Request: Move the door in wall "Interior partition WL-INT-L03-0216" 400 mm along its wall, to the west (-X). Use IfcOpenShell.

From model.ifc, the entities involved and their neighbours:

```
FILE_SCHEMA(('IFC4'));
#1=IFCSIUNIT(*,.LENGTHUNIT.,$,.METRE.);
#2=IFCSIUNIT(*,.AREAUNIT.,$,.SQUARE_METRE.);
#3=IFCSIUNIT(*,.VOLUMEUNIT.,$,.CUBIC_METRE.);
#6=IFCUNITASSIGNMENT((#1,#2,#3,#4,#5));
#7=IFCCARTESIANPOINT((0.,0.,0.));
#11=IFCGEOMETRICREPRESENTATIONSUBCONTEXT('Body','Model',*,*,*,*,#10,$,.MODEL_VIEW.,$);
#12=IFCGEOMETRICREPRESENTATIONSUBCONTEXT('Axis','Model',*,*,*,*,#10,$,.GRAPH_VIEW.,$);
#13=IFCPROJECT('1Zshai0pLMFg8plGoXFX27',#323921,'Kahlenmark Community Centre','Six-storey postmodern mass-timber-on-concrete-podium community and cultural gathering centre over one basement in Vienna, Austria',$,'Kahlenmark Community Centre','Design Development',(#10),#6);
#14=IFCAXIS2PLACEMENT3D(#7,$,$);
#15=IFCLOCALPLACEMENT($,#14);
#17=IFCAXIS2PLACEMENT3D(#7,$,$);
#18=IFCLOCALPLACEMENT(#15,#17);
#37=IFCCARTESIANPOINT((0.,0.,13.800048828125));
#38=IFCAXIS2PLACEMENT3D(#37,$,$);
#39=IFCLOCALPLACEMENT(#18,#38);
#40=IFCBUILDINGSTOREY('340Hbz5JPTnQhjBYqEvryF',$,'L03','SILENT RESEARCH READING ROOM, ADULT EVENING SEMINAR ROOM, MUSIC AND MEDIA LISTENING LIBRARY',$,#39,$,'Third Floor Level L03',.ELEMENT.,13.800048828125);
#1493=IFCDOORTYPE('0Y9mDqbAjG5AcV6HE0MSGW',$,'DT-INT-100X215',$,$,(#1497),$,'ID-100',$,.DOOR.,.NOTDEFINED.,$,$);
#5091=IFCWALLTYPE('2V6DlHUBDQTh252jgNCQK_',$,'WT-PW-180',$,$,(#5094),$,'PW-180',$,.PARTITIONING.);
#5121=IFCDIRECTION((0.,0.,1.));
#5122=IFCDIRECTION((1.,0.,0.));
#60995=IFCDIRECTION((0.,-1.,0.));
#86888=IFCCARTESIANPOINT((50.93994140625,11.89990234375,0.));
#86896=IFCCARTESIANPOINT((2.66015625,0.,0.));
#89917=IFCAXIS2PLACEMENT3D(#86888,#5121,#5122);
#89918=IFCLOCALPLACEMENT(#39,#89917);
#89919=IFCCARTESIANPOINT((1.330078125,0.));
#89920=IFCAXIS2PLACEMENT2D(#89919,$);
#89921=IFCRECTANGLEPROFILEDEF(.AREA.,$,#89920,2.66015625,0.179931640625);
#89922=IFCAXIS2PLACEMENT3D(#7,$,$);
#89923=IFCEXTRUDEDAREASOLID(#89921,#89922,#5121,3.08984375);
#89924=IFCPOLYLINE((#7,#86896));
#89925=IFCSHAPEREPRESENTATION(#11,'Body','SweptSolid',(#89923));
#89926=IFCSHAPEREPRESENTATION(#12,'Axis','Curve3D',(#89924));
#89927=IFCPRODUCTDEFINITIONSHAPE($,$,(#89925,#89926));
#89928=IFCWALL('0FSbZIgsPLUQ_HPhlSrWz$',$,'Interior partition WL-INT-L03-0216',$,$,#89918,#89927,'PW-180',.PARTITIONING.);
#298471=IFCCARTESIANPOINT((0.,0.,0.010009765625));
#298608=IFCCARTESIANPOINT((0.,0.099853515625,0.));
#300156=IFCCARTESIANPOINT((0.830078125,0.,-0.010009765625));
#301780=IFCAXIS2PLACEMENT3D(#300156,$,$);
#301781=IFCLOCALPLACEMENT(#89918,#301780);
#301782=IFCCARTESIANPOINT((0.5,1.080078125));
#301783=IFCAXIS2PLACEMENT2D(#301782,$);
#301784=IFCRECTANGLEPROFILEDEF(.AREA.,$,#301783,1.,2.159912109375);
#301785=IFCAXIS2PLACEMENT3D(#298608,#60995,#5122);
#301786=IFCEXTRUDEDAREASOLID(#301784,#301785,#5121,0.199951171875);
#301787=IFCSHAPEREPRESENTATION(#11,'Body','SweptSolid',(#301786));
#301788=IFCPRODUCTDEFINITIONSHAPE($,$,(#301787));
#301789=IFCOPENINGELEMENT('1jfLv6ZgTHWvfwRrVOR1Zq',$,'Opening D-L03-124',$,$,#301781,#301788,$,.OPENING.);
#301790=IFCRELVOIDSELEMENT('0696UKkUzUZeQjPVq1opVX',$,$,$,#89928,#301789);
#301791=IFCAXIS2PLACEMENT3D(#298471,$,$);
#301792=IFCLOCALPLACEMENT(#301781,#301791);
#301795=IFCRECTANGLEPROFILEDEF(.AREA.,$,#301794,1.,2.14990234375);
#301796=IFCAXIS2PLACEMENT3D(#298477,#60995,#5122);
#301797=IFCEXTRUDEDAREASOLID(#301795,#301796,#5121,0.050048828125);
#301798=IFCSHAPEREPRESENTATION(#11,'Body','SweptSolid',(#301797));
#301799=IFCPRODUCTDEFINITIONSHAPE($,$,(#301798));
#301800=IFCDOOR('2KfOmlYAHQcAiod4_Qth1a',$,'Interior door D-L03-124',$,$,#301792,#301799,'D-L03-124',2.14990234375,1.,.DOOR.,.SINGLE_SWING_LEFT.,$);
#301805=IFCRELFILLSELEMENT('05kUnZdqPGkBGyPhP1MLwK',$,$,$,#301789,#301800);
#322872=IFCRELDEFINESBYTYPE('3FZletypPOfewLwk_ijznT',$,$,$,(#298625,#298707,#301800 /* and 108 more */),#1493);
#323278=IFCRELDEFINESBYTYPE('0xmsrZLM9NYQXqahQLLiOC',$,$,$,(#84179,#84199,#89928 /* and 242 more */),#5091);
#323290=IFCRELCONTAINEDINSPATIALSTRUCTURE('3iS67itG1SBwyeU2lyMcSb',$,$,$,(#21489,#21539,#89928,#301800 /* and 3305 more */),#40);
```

```python
import ifcopenshell
import ifcopenshell.api.geometry
import ifcopenshell.util.placement

model = ifcopenshell.open("model.ifc")

door = model.by_id(301800)
opening = door.FillsVoids[0].RelatingOpeningElement
wall = opening.VoidsElements[0].RelatingBuildingElement

wall_matrix = ifcopenshell.util.placement.get_local_placement(wall.ObjectPlacement)
shift = wall_matrix[:3, 0] * -0.4
before = ifcopenshell.util.placement.get_local_placement(door.ObjectPlacement)[:3, 3].copy()

# The door is placed relative to its opening, so it follows when the opening moves.
matrix = ifcopenshell.util.placement.get_local_placement(opening.ObjectPlacement)
matrix[:3, 3] += shift
ifcopenshell.api.geometry.edit_object_placement(
    model, product=opening, matrix=matrix, is_si=False, should_transform_children=True
)

after = ifcopenshell.util.placement.get_local_placement(door.ObjectPlacement)[:3, 3]
print("door moved by", (after - before).round(3) + 0.0)

model.write("model_v2.ifc")
```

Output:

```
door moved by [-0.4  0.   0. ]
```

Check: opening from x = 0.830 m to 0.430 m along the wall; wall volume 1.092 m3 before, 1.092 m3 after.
